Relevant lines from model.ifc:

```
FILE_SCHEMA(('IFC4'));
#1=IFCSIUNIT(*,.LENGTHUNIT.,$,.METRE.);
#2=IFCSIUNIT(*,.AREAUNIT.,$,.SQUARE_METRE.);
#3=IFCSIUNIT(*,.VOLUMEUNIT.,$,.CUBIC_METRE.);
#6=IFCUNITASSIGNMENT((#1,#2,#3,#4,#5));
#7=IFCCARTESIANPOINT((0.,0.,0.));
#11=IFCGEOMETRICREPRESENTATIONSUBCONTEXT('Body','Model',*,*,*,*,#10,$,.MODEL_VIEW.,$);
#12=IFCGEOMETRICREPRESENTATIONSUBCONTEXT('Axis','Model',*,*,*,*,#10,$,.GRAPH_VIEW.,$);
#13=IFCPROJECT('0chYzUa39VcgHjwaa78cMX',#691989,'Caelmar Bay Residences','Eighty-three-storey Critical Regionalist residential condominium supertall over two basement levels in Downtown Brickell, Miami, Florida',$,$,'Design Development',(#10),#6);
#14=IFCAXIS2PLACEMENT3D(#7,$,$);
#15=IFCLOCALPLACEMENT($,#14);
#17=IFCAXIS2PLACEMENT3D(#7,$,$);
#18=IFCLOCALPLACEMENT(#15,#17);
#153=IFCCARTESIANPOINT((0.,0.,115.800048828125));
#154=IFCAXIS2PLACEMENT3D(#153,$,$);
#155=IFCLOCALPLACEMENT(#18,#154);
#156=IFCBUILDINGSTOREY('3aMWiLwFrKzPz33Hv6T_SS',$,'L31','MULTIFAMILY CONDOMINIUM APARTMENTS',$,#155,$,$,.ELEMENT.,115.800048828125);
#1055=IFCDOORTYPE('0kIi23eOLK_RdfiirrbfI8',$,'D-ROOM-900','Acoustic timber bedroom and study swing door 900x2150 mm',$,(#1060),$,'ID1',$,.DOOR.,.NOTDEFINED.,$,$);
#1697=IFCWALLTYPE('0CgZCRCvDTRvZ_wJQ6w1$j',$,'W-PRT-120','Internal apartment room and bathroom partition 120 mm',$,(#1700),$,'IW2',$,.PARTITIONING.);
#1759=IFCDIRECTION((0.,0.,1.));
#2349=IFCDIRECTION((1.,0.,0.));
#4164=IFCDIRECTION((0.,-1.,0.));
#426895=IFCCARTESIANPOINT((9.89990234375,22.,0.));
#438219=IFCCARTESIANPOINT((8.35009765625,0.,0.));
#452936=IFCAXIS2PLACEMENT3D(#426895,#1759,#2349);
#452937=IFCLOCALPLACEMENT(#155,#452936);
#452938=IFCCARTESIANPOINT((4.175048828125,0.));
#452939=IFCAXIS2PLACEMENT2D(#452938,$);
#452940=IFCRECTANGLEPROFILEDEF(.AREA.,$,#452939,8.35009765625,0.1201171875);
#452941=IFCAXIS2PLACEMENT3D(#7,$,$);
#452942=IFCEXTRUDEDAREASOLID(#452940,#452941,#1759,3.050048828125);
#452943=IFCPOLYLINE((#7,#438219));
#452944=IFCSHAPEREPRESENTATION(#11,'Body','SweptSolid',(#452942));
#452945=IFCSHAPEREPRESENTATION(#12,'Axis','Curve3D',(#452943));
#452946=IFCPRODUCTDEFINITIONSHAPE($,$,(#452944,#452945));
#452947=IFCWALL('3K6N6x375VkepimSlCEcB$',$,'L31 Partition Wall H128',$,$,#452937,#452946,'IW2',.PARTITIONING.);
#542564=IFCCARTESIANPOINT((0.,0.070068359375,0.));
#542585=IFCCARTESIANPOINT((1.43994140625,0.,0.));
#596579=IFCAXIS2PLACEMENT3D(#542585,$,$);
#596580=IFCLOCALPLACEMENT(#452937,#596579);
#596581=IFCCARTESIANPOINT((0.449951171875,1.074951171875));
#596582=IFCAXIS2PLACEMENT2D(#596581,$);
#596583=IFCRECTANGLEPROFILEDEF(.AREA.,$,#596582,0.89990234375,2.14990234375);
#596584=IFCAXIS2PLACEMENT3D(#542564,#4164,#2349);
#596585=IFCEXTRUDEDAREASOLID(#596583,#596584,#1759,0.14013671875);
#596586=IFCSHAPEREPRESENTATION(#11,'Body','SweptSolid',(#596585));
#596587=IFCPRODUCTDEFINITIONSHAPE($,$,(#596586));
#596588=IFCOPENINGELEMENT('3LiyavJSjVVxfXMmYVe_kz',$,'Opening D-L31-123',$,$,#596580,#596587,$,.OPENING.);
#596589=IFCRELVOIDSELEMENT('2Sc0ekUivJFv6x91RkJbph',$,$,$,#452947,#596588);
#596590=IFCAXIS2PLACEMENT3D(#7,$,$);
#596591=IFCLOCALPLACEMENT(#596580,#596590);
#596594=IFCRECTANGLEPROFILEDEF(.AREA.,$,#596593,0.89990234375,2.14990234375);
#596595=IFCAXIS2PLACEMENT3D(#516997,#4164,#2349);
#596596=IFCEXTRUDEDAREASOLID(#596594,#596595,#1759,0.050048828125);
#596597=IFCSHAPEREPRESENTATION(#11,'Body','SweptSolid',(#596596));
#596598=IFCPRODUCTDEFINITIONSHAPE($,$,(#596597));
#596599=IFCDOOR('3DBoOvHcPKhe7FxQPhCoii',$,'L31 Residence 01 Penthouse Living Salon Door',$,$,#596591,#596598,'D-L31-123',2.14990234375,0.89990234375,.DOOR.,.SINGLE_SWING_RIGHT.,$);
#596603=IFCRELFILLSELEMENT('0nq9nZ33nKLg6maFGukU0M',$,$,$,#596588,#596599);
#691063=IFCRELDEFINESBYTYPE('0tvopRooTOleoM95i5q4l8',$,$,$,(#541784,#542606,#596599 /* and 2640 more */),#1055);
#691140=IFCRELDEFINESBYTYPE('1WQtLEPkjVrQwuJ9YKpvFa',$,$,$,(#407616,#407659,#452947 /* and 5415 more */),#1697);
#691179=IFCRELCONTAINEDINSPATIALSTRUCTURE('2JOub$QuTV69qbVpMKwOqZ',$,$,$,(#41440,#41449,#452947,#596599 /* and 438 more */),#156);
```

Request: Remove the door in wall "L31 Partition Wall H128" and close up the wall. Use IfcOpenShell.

```python
import ifcopenshell
import ifcopenshell.api.feature
import ifcopenshell.api.root
import ifcopenshell.geom
import ifcopenshell.util.shape

model = ifcopenshell.open("model.ifc")
settings = ifcopenshell.geom.settings()


def volume(element):
    """Net volume in cubic metres, openings subtracted."""
    shape = ifcopenshell.geom.create_shape(settings, element)
    return ifcopenshell.util.shape.get_volume(shape.geometry)


door = model.by_guid("3DBoOvHcPKhe7FxQPhCoii")
opening = door.FillsVoids[0].RelatingOpeningElement
wall = opening.VoidsElements[0].RelatingBuildingElement
before = volume(wall)

ifcopenshell.api.root.remove_product(model, product=door)
ifcopenshell.api.feature.remove_feature(model, feature=opening)

after = volume(wall)

print(f"wall volume {before:.3f} -> {after:.3f} m3")

model.write("model_v2.ifc")
```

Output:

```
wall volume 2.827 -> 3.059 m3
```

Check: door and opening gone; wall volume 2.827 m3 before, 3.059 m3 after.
